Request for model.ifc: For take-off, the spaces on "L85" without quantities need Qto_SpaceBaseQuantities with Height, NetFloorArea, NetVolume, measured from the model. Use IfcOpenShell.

First a look at what the model holds.

```python
import ifcopenshell
import ifcopenshell.util.element
import ifcopenshell.util.unit

model = ifcopenshell.open("model.ifc")
print(model.schema)
for unit_type in ("LENGTHUNIT", "AREAUNIT", "VOLUMEUNIT"):
    print(unit_type, ifcopenshell.util.unit.calculate_unit_scale(model, unit_type))
storey = next(s for s in model.by_type("IfcBuildingStorey") if s.Name == "L85")
spaces = [e for e in ifcopenshell.util.element.get_decomposition(storey) if e.is_a("IfcSpace")]
for e in sorted(spaces, key=lambda e: e.id()):
    print(e.id(), e.is_a(), e.Name, list(ifcopenshell.util.element.get_psets(e, qtos_only=True)), sep=" | ")
```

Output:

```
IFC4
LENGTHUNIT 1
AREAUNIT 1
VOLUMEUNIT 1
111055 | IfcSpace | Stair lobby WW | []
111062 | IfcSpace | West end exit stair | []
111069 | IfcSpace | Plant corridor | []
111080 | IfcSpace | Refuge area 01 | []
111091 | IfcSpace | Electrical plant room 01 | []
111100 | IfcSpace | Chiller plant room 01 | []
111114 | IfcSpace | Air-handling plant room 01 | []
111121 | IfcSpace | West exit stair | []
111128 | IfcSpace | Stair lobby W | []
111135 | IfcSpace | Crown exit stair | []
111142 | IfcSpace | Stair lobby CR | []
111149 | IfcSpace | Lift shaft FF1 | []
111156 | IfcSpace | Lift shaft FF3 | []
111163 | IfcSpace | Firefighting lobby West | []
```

```python
import ifcopenshell
import ifcopenshell.api.pset
import ifcopenshell.geom
import ifcopenshell.util.element
import ifcopenshell.util.shape
import ifcopenshell.util.unit

model = ifcopenshell.open("model.ifc")
unit_scale = ifcopenshell.util.unit.calculate_unit_scale(model)
area_scale = ifcopenshell.util.unit.calculate_unit_scale(model, "AREAUNIT")
volume_scale = ifcopenshell.util.unit.calculate_unit_scale(model, "VOLUMEUNIT")
settings = ifcopenshell.geom.settings()

storey = next(s for s in model.by_type("IfcBuildingStorey") if s.Name == "L85")
spaces = [e for e in ifcopenshell.util.element.get_decomposition(storey) if e.is_a("IfcSpace")]

for e in sorted(spaces, key=lambda e: e.id()):
    if ifcopenshell.util.element.get_psets(e, qtos_only=True, should_inherit=False):
        continue
    # Geometry comes back in metres, in the element's own axes.
    shape = ifcopenshell.geom.create_shape(settings, e)
    values = {
        "Height": ifcopenshell.util.shape.get_z(shape.geometry) / unit_scale,
        "NetFloorArea": ifcopenshell.util.shape.get_footprint_area(shape.geometry) / area_scale,
        "NetVolume": ifcopenshell.util.shape.get_volume(shape.geometry) / volume_scale,
    }
    qto = ifcopenshell.api.pset.add_qto(model, product=e, name="Qto_SpaceBaseQuantities")
    ifcopenshell.api.pset.edit_qto(model, qto=qto, properties=values)
    print(e.id(), {k: round(v, 3) for k, v in values.items()})

model.write("model_updated.ifc")
```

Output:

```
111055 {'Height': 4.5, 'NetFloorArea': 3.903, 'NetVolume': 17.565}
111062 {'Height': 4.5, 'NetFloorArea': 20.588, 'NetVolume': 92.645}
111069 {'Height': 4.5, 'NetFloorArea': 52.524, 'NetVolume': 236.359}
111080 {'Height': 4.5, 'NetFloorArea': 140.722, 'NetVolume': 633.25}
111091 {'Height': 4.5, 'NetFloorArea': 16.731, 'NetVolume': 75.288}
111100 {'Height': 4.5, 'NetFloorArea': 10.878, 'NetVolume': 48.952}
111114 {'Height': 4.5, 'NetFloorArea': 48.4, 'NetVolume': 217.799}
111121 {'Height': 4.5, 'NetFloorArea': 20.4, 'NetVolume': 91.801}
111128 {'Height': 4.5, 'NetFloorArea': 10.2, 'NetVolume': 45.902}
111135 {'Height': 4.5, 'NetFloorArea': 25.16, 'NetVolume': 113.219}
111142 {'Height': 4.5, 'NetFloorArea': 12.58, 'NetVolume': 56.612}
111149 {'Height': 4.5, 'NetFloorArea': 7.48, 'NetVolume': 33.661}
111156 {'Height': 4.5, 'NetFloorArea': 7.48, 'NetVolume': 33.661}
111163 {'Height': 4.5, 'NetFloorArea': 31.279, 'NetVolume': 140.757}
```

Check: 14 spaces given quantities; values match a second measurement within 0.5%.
